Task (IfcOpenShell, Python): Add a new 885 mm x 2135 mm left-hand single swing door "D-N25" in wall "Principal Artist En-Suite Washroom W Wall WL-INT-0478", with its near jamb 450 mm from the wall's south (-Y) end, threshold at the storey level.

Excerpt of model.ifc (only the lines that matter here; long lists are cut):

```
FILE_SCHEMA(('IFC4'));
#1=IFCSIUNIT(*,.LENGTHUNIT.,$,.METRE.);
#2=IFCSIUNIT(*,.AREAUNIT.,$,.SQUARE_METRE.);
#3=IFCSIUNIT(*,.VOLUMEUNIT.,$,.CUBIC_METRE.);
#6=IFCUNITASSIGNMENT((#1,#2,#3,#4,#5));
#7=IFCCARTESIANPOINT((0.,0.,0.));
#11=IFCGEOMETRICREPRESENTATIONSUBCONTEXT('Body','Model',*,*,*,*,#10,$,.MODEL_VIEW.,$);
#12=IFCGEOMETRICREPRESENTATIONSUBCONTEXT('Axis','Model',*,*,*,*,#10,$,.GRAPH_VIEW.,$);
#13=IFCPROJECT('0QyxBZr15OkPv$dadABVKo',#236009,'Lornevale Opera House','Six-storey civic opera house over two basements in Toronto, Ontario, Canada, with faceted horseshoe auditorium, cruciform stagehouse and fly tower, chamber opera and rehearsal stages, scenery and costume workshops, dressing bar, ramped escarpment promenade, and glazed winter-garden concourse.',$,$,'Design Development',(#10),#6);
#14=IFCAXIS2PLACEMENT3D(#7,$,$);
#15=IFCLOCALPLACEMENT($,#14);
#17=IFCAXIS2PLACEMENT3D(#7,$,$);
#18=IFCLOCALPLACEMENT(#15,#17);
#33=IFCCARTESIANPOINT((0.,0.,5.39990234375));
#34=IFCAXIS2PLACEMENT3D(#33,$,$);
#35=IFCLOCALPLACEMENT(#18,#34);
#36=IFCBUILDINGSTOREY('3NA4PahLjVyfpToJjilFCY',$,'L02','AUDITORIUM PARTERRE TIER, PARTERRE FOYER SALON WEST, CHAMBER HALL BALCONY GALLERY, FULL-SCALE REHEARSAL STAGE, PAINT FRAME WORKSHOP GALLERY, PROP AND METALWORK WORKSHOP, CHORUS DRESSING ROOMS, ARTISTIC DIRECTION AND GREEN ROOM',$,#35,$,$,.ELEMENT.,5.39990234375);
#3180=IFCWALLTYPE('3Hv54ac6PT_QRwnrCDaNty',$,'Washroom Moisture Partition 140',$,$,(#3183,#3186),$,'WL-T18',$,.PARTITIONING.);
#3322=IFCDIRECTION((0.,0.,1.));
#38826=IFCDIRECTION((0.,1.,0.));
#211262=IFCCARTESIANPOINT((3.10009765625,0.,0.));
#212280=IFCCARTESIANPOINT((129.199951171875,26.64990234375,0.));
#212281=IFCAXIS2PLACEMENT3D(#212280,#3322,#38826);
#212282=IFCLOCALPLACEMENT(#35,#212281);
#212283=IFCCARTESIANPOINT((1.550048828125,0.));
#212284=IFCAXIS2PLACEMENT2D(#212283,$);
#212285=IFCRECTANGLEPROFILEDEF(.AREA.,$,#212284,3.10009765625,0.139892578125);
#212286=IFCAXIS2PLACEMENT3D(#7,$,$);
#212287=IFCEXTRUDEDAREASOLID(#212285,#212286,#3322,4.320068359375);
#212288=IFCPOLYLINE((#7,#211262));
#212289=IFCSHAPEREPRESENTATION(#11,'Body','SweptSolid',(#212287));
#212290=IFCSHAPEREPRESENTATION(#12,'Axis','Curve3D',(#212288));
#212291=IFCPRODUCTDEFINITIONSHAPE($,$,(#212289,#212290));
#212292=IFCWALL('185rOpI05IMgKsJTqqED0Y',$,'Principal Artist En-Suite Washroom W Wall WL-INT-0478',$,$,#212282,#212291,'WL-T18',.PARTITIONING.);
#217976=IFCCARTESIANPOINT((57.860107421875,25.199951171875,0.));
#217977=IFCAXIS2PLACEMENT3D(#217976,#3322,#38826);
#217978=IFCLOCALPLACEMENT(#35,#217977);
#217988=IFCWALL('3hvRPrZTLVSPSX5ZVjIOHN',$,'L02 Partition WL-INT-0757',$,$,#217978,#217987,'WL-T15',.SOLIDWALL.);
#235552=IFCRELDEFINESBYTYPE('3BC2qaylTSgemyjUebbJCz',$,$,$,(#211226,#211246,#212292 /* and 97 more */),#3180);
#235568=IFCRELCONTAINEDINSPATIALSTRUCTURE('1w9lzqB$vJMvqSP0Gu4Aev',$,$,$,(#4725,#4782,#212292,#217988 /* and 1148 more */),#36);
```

```python
import numpy as np
import ifcopenshell
import ifcopenshell.api.feature
import ifcopenshell.api.geometry
import ifcopenshell.api.root
import ifcopenshell.api.spatial
import ifcopenshell.geom
import ifcopenshell.util.element
import ifcopenshell.util.placement
import ifcopenshell.util.representation
import ifcopenshell.util.shape
import ifcopenshell.util.unit

model = ifcopenshell.open("model.ifc")
unit_scale = ifcopenshell.util.unit.calculate_unit_scale(model)
settings = ifcopenshell.geom.settings()


def volume(element):
    """Net volume in cubic metres, openings subtracted."""
    shape = ifcopenshell.geom.create_shape(settings, element)
    return ifcopenshell.util.shape.get_volume(shape.geometry)


wall = model.by_guid("185rOpI05IMgKsJTqqED0Y")
storey = ifcopenshell.util.element.get_container(wall, ifc_class="IfcBuildingStorey")
context = ifcopenshell.util.representation.get_context(model, "Model", "Body", "MODEL_VIEW")
before = volume(wall)

width, height, from_end, sill = 0.885, 2.135, 0.45, 0.0  # metres

# The wall runs along its own X axis, and the end named is its -X end.
wall_shape = ifcopenshell.geom.create_shape(settings, wall)
x, y, z = ifcopenshell.util.shape.get_vertices(wall_shape.geometry).T
start = x.min() + from_end
face, thickness = float(y.min()), float(y.max() - y.min())
wall_matrix = ifcopenshell.util.placement.get_local_placement(wall.ObjectPlacement)
level = ifcopenshell.util.placement.get_local_placement(storey.ObjectPlacement)[2, 3]


def in_wall(x, y):
    """Placement at x, y metres in the wall's axes, at sill height."""
    matrix = wall_matrix.copy()
    matrix[:, 3] = wall_matrix @ np.array([x / unit_scale, y / unit_scale, 0.0, 1.0])
    matrix[2, 3] = level + sill / unit_scale
    return matrix


# Opening: a box that overshoots both wall faces by 50 mm.
opening = ifcopenshell.api.root.create_entity(model, ifc_class="IfcOpeningElement", predefined_type="OPENING")
box = ifcopenshell.api.geometry.add_wall_representation(
    model, context=context, length=width, height=height, thickness=thickness + 0.1
)
ifcopenshell.api.geometry.assign_representation(model, product=opening, representation=box)
ifcopenshell.api.geometry.edit_object_placement(model, product=opening, matrix=in_wall(start, face - 0.05), is_si=False)
ifcopenshell.api.feature.add_feature(model, feature=opening, element=wall)

door = ifcopenshell.api.root.create_entity(model, ifc_class="IfcDoor", name="D-N25", predefined_type="DOOR")
door.OverallWidth, door.OverallHeight = width / unit_scale, height / unit_scale
door.OperationType = "SINGLE_SWING_LEFT"
body = ifcopenshell.api.geometry.add_door_representation(
    model,
    context=context,
    overall_width=door.OverallWidth,
    overall_height=door.OverallHeight,
    operation_type="SINGLE_SWING_LEFT",
    lining_properties={"LiningDepth": thickness / unit_scale, "ThresholdDepth": thickness / unit_scale},
)
ifcopenshell.api.geometry.assign_representation(model, product=door, representation=body)
ifcopenshell.api.spatial.assign_container(model, products=[door], relating_structure=storey)
ifcopenshell.api.feature.add_filling(model, opening=opening, element=door)

# The lining spans the wall, so the door starts at the wall face.
ifcopenshell.api.geometry.edit_object_placement(model, product=door, matrix=in_wall(start, face), is_si=False)

after = volume(wall)

print(f"wall volume {before:.3f} -> {after:.3f} m3")

model.write("model_rev.ifc")
```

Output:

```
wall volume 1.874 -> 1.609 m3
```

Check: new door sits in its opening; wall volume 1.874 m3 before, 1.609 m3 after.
